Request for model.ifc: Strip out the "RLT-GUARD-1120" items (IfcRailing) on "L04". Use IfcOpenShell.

First a look at what the model holds.

```python
import ifcopenshell
import ifcopenshell.util.element

model = ifcopenshell.open("model.ifc")
print(model.schema)
storey = next(s for s in model.by_type("IfcBuildingStorey") if s.Name == "L04")
railings = [e for e in ifcopenshell.util.element.get_decomposition(storey) if e.is_a("IfcRailing")]
seen = {}
for e in railings:
    element_type = ifcopenshell.util.element.get_type(e)
    name = element_type.Name if element_type not in (None, e) else None
    seen[name] = seen.get(name, 0) + 1
for name, count in sorted(seen.items(), key=str):
    print(count, "x", name)
```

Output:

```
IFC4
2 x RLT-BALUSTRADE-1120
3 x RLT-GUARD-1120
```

```python
import ifcopenshell
import ifcopenshell.api.root
import ifcopenshell.util.element

model = ifcopenshell.open("model.ifc")

storey = next(s for s in model.by_type("IfcBuildingStorey") if s.Name == "L04")
railings = [e for e in ifcopenshell.util.element.get_decomposition(storey) if e.is_a("IfcRailing")]
targets = [e for e in railings if (t := ifcopenshell.util.element.get_type(e)) not in (None, e) and t.Name == "RLT-GUARD-1120"]

for e in targets:
    ifcopenshell.api.root.remove_product(model, product=e)
print(len(targets), "removed")

model.write("model_v2.ifc")
```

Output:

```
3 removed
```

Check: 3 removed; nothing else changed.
